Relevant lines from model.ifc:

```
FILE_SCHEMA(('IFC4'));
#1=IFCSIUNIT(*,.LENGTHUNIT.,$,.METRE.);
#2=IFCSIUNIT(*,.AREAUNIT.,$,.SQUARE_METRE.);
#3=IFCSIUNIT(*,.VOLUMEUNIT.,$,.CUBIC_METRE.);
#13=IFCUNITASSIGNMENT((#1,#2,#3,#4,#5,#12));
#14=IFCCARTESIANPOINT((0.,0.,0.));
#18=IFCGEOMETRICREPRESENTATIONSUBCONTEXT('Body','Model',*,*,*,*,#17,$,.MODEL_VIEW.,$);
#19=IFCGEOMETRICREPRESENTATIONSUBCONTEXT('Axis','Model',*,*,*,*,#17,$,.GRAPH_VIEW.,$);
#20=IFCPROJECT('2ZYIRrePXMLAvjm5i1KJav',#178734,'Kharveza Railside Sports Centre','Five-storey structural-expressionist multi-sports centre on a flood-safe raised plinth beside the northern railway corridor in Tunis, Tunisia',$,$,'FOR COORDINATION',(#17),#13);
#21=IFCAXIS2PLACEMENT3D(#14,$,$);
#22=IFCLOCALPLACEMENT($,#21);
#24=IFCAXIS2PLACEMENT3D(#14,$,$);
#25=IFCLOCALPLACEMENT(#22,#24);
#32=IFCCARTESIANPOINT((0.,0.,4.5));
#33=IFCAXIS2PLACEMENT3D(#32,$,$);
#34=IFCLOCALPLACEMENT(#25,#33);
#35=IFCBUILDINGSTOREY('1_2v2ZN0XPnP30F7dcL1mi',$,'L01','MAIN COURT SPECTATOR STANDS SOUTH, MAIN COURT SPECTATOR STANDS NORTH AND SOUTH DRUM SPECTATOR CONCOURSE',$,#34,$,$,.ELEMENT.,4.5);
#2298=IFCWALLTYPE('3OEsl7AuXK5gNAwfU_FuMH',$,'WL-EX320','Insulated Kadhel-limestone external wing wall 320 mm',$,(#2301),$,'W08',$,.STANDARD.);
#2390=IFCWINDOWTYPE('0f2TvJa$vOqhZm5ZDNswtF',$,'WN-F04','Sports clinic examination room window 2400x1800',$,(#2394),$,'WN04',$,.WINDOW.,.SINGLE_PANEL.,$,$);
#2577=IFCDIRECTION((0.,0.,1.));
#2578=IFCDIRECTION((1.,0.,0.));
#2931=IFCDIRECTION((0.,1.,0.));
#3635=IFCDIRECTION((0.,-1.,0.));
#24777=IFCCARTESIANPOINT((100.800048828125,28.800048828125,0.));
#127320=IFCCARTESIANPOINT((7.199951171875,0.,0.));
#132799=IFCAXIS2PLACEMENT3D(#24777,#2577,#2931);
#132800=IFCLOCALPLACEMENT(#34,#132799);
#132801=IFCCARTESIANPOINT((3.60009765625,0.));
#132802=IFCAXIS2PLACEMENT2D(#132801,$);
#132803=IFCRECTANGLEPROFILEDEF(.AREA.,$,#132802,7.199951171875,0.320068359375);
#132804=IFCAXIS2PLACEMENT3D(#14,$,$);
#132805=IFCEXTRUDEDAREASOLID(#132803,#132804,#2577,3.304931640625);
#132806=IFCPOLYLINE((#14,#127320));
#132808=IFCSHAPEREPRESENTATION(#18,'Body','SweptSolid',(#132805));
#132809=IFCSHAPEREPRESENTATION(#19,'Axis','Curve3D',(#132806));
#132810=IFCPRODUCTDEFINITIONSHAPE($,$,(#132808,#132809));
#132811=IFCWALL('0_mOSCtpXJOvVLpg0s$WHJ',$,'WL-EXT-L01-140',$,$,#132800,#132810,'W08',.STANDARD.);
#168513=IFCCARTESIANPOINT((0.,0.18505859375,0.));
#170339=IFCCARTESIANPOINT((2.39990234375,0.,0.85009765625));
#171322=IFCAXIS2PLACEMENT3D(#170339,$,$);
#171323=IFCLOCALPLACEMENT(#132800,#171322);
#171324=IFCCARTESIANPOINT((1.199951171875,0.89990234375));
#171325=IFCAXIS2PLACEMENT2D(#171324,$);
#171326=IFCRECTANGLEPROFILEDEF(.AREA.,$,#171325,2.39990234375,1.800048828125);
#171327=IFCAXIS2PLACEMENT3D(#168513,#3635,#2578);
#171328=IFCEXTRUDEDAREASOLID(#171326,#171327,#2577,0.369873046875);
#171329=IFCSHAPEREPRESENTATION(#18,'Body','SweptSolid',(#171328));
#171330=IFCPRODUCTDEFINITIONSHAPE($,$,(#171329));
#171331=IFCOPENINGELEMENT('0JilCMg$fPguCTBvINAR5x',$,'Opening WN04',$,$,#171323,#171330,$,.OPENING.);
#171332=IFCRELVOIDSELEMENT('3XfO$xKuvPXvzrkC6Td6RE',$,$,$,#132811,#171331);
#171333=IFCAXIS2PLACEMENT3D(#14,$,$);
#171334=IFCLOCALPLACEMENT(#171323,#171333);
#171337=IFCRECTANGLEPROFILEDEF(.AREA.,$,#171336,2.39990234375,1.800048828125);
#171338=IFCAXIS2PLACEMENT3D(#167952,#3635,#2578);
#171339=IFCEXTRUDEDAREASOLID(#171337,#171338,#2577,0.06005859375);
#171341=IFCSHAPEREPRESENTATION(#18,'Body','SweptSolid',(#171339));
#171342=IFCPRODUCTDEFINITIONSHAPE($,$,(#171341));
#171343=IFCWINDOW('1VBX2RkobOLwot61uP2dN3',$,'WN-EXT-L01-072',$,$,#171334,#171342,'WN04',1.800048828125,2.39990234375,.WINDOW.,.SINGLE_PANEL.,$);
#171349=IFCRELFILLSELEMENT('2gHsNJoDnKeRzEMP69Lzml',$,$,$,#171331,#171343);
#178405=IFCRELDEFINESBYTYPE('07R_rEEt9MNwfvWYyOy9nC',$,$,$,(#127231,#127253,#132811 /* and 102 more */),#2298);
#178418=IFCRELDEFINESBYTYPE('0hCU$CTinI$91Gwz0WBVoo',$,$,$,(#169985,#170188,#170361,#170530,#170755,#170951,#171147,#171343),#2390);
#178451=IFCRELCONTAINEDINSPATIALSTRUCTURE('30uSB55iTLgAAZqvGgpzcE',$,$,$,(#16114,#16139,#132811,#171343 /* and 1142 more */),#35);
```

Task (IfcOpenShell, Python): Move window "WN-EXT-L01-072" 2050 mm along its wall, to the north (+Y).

```python
import ifcopenshell
import ifcopenshell.api.geometry
import ifcopenshell.util.placement
import ifcopenshell.util.unit

model = ifcopenshell.open("model.ifc")
unit_scale = ifcopenshell.util.unit.calculate_unit_scale(model)

window = model.by_guid("1VBX2RkobOLwot61uP2dN3")
opening = window.FillsVoids[0].RelatingOpeningElement
wall = opening.VoidsElements[0].RelatingBuildingElement

wall_matrix = ifcopenshell.util.placement.get_local_placement(wall.ObjectPlacement)
shift = wall_matrix[:3, 0] * 2.05 / unit_scale
before = ifcopenshell.util.placement.get_local_placement(window.ObjectPlacement)[:3, 3].copy()

# The window is placed relative to its opening, so it follows when the opening moves.
matrix = ifcopenshell.util.placement.get_local_placement(opening.ObjectPlacement)
matrix[:3, 3] += shift
ifcopenshell.api.geometry.edit_object_placement(
    model, product=opening, matrix=matrix, is_si=False, should_transform_children=True
)

after = ifcopenshell.util.placement.get_local_placement(window.ObjectPlacement)[:3, 3]
print("window moved by", (after - before).round(3) + 0.0)

model.write("model_v2.ifc")
```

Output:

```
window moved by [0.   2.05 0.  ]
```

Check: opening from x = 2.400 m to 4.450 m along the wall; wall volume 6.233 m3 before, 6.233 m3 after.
